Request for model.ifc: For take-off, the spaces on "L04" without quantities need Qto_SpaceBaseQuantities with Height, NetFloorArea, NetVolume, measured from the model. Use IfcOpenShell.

First a look at what the model holds.

```python
import ifcopenshell
import ifcopenshell.util.element
import ifcopenshell.util.unit

model = ifcopenshell.open("model.ifc")
print(model.schema)
for unit_type in ("LENGTHUNIT", "AREAUNIT", "VOLUMEUNIT"):
    print(unit_type, ifcopenshell.util.unit.calculate_unit_scale(model, unit_type))
storey = next(s for s in model.by_type("IfcBuildingStorey") if s.Name == "L04")
spaces = [e for e in ifcopenshell.util.element.get_decomposition(storey) if e.is_a("IfcSpace")]
for e in sorted(spaces, key=lambda e: e.id()):
    print(e.id(), e.is_a(), e.Name, list(ifcopenshell.util.element.get_psets(e, qtos_only=True)), sep=" | ")
```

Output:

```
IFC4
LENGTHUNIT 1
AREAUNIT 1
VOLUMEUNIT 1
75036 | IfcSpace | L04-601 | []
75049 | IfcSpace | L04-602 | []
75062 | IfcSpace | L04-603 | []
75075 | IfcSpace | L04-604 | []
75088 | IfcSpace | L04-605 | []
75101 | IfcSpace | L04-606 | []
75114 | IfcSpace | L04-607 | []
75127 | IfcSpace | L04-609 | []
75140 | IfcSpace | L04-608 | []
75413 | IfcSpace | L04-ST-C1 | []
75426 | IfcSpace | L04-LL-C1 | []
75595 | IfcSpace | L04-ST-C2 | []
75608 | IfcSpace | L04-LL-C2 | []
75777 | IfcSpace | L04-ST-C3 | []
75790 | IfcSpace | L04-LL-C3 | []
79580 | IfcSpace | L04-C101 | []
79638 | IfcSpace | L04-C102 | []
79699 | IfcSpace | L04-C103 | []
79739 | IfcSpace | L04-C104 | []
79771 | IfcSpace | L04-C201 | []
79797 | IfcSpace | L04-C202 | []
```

```python
import ifcopenshell
import ifcopenshell.api.pset
import ifcopenshell.geom
import ifcopenshell.util.element
import ifcopenshell.util.shape
import ifcopenshell.util.unit

model = ifcopenshell.open("model.ifc")
unit_scale = ifcopenshell.util.unit.calculate_unit_scale(model)
area_scale = ifcopenshell.util.unit.calculate_unit_scale(model, "AREAUNIT")
volume_scale = ifcopenshell.util.unit.calculate_unit_scale(model, "VOLUMEUNIT")
settings = ifcopenshell.geom.settings()

storey = next(s for s in model.by_type("IfcBuildingStorey") if s.Name == "L04")
spaces = [e for e in ifcopenshell.util.element.get_decomposition(storey) if e.is_a("IfcSpace")]

for e in sorted(spaces, key=lambda e: e.id()):
    if ifcopenshell.util.element.get_psets(e, qtos_only=True, should_inherit=False):
        continue
    # Geometry comes back in metres, in the element's own axes.
    shape = ifcopenshell.geom.create_shape(settings, e)
    values = {
        "Height": ifcopenshell.util.shape.get_z(shape.geometry) / unit_scale,
        "NetFloorArea": ifcopenshell.util.shape.get_footprint_area(shape.geometry) / area_scale,
        "NetVolume": ifcopenshell.util.shape.get_volume(shape.geometry) / volume_scale,
    }
    qto = ifcopenshell.api.pset.add_qto(model, product=e, name="Qto_SpaceBaseQuantities")
    ifcopenshell.api.pset.edit_qto(model, qto=qto, properties=values)
    print(e.id(), {k: round(v, 3) for k, v in values.items()})

model.write("model_edited.ifc")
```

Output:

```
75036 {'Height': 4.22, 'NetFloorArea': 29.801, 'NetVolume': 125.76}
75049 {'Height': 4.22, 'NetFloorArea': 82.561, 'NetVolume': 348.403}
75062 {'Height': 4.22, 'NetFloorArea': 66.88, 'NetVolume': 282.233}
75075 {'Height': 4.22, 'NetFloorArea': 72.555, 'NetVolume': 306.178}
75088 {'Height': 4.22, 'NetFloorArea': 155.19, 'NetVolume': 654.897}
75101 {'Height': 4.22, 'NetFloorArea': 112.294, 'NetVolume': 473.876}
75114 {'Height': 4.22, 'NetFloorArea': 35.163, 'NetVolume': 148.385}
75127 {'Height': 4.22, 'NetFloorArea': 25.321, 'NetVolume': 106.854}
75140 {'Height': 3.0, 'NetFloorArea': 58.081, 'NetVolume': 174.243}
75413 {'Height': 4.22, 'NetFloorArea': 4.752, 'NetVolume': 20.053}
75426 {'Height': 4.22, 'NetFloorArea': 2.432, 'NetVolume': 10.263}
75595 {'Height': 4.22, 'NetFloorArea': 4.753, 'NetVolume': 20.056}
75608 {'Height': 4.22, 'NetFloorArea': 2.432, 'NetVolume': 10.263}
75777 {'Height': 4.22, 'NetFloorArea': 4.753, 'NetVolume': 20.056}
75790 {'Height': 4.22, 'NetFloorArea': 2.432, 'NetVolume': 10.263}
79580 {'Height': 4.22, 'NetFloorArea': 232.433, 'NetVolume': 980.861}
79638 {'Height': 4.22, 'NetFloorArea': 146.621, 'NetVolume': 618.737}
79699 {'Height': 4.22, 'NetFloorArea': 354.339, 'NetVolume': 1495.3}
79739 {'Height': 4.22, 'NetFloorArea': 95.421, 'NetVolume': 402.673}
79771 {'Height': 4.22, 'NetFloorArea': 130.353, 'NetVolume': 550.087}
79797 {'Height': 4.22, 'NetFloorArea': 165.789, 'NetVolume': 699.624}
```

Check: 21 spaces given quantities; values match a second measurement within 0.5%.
